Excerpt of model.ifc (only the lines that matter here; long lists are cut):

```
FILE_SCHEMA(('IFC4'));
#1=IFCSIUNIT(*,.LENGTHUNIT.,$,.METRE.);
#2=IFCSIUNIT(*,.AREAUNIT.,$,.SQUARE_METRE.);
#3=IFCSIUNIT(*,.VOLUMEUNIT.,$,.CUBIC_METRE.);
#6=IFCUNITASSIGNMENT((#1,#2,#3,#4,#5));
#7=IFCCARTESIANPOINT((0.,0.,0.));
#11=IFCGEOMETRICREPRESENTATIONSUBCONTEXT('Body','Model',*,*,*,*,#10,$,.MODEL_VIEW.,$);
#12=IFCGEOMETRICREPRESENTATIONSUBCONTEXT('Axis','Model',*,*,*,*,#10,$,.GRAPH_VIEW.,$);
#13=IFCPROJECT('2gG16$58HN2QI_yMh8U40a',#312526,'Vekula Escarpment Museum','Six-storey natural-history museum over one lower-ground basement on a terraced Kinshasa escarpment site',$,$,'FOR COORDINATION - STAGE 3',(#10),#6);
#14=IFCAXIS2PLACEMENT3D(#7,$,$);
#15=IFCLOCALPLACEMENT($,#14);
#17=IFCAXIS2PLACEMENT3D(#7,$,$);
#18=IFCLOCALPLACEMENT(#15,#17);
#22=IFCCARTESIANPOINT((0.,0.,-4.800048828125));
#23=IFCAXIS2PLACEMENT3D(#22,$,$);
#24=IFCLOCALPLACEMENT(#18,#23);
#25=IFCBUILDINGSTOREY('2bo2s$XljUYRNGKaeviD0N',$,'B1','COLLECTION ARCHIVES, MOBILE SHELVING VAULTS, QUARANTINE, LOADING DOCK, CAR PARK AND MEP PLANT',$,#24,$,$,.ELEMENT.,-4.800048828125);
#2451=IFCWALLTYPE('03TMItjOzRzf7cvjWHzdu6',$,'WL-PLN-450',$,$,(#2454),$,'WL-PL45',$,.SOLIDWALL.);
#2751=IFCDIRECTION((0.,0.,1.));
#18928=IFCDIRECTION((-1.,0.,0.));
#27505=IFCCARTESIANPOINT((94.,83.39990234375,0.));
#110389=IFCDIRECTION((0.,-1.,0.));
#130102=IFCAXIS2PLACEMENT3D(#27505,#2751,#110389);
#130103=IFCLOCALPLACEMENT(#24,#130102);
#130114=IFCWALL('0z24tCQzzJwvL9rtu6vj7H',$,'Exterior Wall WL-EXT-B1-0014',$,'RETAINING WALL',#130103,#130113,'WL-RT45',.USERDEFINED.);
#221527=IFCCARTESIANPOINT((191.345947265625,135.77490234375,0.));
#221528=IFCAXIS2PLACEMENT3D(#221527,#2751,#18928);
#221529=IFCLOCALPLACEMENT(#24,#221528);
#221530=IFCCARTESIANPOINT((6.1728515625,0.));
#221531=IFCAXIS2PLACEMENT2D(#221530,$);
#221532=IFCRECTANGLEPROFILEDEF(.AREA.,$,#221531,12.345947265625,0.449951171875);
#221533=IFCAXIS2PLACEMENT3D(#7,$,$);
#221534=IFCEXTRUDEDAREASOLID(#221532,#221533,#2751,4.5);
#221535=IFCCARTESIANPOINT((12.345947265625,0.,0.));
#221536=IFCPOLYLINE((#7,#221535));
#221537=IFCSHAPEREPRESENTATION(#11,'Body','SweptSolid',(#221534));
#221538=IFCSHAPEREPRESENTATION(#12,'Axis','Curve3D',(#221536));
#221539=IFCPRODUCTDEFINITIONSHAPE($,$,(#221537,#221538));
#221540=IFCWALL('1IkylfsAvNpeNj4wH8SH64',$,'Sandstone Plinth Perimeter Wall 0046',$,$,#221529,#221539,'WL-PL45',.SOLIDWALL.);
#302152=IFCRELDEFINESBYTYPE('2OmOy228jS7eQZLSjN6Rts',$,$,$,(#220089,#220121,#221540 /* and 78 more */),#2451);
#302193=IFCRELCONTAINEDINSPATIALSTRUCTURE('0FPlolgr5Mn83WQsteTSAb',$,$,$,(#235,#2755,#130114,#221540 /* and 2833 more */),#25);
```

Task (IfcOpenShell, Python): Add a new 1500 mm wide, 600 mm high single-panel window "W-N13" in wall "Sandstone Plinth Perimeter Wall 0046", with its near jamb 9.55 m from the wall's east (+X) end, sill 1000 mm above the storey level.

```python
import numpy as np
import ifcopenshell
import ifcopenshell.api.feature
import ifcopenshell.api.geometry
import ifcopenshell.api.root
import ifcopenshell.api.spatial
import ifcopenshell.geom
import ifcopenshell.util.element
import ifcopenshell.util.placement
import ifcopenshell.util.representation
import ifcopenshell.util.shape
import ifcopenshell.util.unit

model = ifcopenshell.open("model.ifc")
unit_scale = ifcopenshell.util.unit.calculate_unit_scale(model)
settings = ifcopenshell.geom.settings()


def volume(element):
    """Net volume in cubic metres, openings subtracted."""
    shape = ifcopenshell.geom.create_shape(settings, element)
    return ifcopenshell.util.shape.get_volume(shape.geometry)


wall = model.by_guid("1IkylfsAvNpeNj4wH8SH64")
storey = ifcopenshell.util.element.get_container(wall, ifc_class="IfcBuildingStorey")
context = ifcopenshell.util.representation.get_context(model, "Model", "Body", "MODEL_VIEW")
before = volume(wall)

width, height, from_end, sill = 1.5, 0.6, 9.55, 1  # metres

# The wall runs along its own X axis, and the end named is its -X end.
wall_shape = ifcopenshell.geom.create_shape(settings, wall)
x, y, z = ifcopenshell.util.shape.get_vertices(wall_shape.geometry).T
start = x.min() + from_end
face, thickness = float(y.min()), float(y.max() - y.min())
wall_matrix = ifcopenshell.util.placement.get_local_placement(wall.ObjectPlacement)
level = ifcopenshell.util.placement.get_local_placement(storey.ObjectPlacement)[2, 3]


def in_wall(x, y):
    """Placement at x, y metres in the wall's axes, at sill height."""
    matrix = wall_matrix.copy()
    matrix[:, 3] = wall_matrix @ np.array([x / unit_scale, y / unit_scale, 0.0, 1.0])
    matrix[2, 3] = level + sill / unit_scale
    return matrix


# Opening: a box that overshoots both wall faces by 50 mm.
opening = ifcopenshell.api.root.create_entity(model, ifc_class="IfcOpeningElement", predefined_type="OPENING")
box = ifcopenshell.api.geometry.add_wall_representation(
    model, context=context, length=width, height=height, thickness=thickness + 0.1
)
ifcopenshell.api.geometry.assign_representation(model, product=opening, representation=box)
ifcopenshell.api.geometry.edit_object_placement(model, product=opening, matrix=in_wall(start, face - 0.05), is_si=False)
ifcopenshell.api.feature.add_feature(model, feature=opening, element=wall)

window = ifcopenshell.api.root.create_entity(model, ifc_class="IfcWindow", name="W-N13", predefined_type="WINDOW")
window.OverallWidth, window.OverallHeight = width / unit_scale, height / unit_scale
window.PartitioningType = "SINGLE_PANEL"
body = ifcopenshell.api.geometry.add_window_representation(
    model,
    context=context,
    overall_width=window.OverallWidth,
    overall_height=window.OverallHeight,
    partition_type="SINGLE_PANEL",
)
ifcopenshell.api.geometry.assign_representation(model, product=window, representation=body)
ifcopenshell.api.spatial.assign_container(model, products=[window], relating_structure=storey)
ifcopenshell.api.feature.add_filling(model, opening=opening, element=window)

# Centre the window in the wall's thickness.
ifcopenshell.api.geometry.edit_object_placement(model, product=window, matrix=in_wall(start, face), is_si=False)
window_shape = ifcopenshell.geom.create_shape(settings, window)
depth = ifcopenshell.util.shape.get_vertices(window_shape.geometry)[:, 1]
offset = face + thickness / 2 - (depth.min() + depth.max()) / 2
ifcopenshell.api.geometry.edit_object_placement(model, product=window, matrix=in_wall(start, offset), is_si=False)

after = volume(wall)

print(f"wall volume {before:.3f} -> {after:.3f} m3")

model.write("model_v2.ifc")
```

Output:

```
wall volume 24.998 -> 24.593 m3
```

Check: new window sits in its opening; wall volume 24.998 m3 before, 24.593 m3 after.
